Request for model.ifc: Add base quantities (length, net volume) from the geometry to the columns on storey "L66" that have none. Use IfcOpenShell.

First a look at what the model holds.

```python
import ifcopenshell
import ifcopenshell.util.element
import ifcopenshell.util.unit

model = ifcopenshell.open("model.ifc")
print(model.schema)
for unit_type in ("LENGTHUNIT", "AREAUNIT", "VOLUMEUNIT"):
    print(unit_type, ifcopenshell.util.unit.calculate_unit_scale(model, unit_type))
storey = next(s for s in model.by_type("IfcBuildingStorey") if s.Name == "L66")
columns = [e for e in ifcopenshell.util.element.get_decomposition(storey) if e.is_a("IfcColumn")]
for e in sorted(columns, key=lambda e: e.id()):
    print(e.id(), e.is_a(), e.Name, list(ifcopenshell.util.element.get_psets(e, qtos_only=True)), sep=" | ")
```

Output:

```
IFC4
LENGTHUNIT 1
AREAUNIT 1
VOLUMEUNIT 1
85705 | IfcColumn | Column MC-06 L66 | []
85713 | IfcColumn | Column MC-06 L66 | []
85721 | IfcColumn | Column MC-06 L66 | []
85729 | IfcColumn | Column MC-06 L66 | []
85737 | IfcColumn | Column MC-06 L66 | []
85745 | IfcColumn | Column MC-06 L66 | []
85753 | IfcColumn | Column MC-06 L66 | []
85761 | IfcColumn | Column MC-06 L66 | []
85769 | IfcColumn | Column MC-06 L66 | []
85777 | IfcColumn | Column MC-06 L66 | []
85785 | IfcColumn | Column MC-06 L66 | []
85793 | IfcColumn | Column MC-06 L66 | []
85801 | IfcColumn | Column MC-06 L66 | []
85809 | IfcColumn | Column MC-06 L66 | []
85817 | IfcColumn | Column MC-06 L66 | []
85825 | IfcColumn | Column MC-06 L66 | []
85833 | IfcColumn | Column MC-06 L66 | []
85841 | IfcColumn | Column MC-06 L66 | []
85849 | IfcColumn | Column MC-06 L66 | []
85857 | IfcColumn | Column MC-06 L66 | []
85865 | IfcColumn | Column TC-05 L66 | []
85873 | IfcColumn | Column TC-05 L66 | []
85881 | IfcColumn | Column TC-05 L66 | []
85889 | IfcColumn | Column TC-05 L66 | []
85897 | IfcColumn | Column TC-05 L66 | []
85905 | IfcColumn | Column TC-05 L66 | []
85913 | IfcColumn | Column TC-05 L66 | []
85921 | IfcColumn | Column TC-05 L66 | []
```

```python
import ifcopenshell
import ifcopenshell.api.pset
import ifcopenshell.geom
import ifcopenshell.util.element
import ifcopenshell.util.shape
import ifcopenshell.util.unit

model = ifcopenshell.open("model.ifc")
unit_scale = ifcopenshell.util.unit.calculate_unit_scale(model)
volume_scale = ifcopenshell.util.unit.calculate_unit_scale(model, "VOLUMEUNIT")
settings = ifcopenshell.geom.settings()

storey = next(s for s in model.by_type("IfcBuildingStorey") if s.Name == "L66")
columns = [e for e in ifcopenshell.util.element.get_decomposition(storey) if e.is_a("IfcColumn")]

for e in sorted(columns, key=lambda e: e.id()):
    if ifcopenshell.util.element.get_psets(e, qtos_only=True, should_inherit=False):
        continue
    # Geometry comes back in metres, in the element's own axes.
    shape = ifcopenshell.geom.create_shape(settings, e)
    values = {
        "Length": ifcopenshell.util.shape.get_z(shape.geometry) / unit_scale,
        "NetVolume": ifcopenshell.util.shape.get_volume(shape.geometry) / volume_scale,
    }
    qto = ifcopenshell.api.pset.add_qto(model, product=e, name="Qto_ColumnBaseQuantities")
    ifcopenshell.api.pset.edit_qto(model, qto=qto, properties=values)
    print(e.id(), {k: round(v, 3) for k, v in values.items()})

model.write("model-out.ifc")
```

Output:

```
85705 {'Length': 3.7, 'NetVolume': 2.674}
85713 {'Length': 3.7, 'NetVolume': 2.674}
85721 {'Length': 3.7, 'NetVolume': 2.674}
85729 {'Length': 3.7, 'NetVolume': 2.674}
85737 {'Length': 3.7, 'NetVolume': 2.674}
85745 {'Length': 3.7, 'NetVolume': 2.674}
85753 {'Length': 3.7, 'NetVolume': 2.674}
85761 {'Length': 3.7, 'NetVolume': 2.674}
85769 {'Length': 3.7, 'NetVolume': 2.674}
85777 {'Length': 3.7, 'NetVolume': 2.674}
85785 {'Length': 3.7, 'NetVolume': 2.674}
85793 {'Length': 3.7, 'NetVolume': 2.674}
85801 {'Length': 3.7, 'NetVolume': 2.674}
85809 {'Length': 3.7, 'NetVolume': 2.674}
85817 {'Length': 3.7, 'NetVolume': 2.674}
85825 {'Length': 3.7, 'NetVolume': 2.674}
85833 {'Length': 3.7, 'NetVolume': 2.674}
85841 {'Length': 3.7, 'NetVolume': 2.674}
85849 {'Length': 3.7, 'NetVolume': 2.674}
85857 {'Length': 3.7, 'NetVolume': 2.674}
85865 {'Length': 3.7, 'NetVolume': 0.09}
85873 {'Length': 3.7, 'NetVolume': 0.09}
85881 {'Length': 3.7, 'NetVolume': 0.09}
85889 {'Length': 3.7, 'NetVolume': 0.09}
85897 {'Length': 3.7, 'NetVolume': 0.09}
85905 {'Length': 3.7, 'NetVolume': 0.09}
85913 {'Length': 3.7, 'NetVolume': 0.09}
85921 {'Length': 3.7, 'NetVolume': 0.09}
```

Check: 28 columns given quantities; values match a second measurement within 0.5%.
